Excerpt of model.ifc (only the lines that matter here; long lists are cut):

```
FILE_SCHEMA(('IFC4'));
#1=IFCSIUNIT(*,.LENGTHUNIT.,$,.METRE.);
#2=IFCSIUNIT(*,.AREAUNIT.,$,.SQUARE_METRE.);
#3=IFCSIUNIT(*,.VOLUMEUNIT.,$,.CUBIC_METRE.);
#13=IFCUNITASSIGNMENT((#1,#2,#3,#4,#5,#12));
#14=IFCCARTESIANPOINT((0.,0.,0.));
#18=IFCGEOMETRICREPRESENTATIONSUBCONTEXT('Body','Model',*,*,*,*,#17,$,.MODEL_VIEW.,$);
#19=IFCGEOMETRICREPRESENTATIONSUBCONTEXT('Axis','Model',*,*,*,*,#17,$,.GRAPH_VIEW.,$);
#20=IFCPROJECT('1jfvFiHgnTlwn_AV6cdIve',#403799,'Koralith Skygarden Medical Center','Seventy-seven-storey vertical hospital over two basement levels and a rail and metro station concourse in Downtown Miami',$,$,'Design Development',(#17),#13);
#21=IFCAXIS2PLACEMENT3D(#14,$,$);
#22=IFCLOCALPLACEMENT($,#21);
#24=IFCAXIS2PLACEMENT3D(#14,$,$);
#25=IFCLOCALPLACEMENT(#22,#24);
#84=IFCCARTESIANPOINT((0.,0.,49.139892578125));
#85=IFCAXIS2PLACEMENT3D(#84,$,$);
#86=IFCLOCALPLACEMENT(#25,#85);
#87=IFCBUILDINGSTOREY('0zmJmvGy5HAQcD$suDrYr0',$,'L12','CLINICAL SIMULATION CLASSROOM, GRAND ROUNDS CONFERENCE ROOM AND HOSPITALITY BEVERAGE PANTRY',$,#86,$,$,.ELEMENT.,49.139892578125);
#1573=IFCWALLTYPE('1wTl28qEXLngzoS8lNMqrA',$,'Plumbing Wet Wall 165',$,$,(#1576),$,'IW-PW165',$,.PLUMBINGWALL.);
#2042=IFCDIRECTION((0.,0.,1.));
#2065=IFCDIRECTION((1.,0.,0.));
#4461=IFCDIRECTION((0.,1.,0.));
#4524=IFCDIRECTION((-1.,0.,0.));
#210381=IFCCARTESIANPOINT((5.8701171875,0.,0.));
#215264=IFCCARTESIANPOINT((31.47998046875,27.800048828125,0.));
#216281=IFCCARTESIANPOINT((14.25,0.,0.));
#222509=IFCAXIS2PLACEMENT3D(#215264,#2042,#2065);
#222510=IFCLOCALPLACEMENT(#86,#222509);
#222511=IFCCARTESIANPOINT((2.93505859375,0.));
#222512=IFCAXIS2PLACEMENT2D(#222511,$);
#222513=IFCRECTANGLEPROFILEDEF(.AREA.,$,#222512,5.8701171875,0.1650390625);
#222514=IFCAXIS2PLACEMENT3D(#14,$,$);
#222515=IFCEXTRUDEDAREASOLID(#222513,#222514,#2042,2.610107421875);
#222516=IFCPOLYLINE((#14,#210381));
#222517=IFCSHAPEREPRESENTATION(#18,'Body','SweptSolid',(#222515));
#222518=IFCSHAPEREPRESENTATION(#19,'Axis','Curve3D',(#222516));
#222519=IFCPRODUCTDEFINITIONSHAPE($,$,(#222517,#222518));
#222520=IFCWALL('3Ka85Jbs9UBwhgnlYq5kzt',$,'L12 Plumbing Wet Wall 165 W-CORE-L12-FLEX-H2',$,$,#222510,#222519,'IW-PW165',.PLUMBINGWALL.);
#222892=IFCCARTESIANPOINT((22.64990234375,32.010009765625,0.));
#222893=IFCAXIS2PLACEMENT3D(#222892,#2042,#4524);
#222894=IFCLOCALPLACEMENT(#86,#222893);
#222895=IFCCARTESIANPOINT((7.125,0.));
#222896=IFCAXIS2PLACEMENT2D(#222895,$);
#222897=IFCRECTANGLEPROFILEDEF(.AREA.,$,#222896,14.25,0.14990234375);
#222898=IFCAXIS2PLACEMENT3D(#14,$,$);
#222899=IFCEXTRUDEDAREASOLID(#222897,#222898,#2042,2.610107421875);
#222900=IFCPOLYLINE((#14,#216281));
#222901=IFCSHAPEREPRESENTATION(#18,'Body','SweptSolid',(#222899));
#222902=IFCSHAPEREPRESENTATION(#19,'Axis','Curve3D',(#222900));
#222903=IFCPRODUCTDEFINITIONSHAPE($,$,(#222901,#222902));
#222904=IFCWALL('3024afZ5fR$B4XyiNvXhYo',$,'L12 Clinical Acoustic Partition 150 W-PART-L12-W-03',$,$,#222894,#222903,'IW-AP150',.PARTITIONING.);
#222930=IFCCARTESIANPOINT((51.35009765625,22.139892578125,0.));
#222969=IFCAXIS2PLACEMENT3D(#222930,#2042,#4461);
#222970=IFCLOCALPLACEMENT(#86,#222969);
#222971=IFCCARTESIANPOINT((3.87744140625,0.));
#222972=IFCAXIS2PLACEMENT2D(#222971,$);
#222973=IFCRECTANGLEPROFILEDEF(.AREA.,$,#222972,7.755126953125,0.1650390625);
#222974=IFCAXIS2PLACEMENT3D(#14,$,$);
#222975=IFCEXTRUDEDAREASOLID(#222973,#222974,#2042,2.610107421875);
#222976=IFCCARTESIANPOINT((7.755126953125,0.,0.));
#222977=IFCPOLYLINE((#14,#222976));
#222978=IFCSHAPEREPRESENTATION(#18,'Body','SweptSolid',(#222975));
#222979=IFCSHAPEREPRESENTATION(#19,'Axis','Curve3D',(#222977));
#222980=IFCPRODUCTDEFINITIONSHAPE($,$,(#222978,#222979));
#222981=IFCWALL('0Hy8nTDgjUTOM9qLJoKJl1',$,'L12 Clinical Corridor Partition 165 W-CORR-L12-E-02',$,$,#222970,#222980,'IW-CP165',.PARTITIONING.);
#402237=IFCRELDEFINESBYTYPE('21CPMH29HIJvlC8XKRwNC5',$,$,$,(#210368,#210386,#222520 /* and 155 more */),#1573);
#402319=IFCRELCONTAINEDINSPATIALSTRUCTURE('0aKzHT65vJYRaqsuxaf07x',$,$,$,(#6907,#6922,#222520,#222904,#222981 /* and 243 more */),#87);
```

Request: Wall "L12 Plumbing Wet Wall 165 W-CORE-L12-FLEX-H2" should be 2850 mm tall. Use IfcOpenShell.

```python
import ifcopenshell
import ifcopenshell.geom
import ifcopenshell.util.representation
import ifcopenshell.util.shape

model = ifcopenshell.open("model.ifc")
settings = ifcopenshell.geom.settings()


def volume(element):
    """Net volume in cubic metres, openings subtracted."""
    shape = ifcopenshell.geom.create_shape(settings, element)
    return ifcopenshell.util.shape.get_volume(shape.geometry)


wall = model.by_guid("3Ka85Jbs9UBwhgnlYq5kzt")
before = volume(wall)

body = ifcopenshell.util.representation.get_representation(wall, "Model", "Body")
solid = body.Items[0]
old_height = solid.Depth
solid.Depth = 2.85
after = volume(wall)

print(f"height {old_height:g} -> {solid.Depth:g}, volume {before:.3f} -> {after:.3f} m3")

model.write("model_updated.ifc")
```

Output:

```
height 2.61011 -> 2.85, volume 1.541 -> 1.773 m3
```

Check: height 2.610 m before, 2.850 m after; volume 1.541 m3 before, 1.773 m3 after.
